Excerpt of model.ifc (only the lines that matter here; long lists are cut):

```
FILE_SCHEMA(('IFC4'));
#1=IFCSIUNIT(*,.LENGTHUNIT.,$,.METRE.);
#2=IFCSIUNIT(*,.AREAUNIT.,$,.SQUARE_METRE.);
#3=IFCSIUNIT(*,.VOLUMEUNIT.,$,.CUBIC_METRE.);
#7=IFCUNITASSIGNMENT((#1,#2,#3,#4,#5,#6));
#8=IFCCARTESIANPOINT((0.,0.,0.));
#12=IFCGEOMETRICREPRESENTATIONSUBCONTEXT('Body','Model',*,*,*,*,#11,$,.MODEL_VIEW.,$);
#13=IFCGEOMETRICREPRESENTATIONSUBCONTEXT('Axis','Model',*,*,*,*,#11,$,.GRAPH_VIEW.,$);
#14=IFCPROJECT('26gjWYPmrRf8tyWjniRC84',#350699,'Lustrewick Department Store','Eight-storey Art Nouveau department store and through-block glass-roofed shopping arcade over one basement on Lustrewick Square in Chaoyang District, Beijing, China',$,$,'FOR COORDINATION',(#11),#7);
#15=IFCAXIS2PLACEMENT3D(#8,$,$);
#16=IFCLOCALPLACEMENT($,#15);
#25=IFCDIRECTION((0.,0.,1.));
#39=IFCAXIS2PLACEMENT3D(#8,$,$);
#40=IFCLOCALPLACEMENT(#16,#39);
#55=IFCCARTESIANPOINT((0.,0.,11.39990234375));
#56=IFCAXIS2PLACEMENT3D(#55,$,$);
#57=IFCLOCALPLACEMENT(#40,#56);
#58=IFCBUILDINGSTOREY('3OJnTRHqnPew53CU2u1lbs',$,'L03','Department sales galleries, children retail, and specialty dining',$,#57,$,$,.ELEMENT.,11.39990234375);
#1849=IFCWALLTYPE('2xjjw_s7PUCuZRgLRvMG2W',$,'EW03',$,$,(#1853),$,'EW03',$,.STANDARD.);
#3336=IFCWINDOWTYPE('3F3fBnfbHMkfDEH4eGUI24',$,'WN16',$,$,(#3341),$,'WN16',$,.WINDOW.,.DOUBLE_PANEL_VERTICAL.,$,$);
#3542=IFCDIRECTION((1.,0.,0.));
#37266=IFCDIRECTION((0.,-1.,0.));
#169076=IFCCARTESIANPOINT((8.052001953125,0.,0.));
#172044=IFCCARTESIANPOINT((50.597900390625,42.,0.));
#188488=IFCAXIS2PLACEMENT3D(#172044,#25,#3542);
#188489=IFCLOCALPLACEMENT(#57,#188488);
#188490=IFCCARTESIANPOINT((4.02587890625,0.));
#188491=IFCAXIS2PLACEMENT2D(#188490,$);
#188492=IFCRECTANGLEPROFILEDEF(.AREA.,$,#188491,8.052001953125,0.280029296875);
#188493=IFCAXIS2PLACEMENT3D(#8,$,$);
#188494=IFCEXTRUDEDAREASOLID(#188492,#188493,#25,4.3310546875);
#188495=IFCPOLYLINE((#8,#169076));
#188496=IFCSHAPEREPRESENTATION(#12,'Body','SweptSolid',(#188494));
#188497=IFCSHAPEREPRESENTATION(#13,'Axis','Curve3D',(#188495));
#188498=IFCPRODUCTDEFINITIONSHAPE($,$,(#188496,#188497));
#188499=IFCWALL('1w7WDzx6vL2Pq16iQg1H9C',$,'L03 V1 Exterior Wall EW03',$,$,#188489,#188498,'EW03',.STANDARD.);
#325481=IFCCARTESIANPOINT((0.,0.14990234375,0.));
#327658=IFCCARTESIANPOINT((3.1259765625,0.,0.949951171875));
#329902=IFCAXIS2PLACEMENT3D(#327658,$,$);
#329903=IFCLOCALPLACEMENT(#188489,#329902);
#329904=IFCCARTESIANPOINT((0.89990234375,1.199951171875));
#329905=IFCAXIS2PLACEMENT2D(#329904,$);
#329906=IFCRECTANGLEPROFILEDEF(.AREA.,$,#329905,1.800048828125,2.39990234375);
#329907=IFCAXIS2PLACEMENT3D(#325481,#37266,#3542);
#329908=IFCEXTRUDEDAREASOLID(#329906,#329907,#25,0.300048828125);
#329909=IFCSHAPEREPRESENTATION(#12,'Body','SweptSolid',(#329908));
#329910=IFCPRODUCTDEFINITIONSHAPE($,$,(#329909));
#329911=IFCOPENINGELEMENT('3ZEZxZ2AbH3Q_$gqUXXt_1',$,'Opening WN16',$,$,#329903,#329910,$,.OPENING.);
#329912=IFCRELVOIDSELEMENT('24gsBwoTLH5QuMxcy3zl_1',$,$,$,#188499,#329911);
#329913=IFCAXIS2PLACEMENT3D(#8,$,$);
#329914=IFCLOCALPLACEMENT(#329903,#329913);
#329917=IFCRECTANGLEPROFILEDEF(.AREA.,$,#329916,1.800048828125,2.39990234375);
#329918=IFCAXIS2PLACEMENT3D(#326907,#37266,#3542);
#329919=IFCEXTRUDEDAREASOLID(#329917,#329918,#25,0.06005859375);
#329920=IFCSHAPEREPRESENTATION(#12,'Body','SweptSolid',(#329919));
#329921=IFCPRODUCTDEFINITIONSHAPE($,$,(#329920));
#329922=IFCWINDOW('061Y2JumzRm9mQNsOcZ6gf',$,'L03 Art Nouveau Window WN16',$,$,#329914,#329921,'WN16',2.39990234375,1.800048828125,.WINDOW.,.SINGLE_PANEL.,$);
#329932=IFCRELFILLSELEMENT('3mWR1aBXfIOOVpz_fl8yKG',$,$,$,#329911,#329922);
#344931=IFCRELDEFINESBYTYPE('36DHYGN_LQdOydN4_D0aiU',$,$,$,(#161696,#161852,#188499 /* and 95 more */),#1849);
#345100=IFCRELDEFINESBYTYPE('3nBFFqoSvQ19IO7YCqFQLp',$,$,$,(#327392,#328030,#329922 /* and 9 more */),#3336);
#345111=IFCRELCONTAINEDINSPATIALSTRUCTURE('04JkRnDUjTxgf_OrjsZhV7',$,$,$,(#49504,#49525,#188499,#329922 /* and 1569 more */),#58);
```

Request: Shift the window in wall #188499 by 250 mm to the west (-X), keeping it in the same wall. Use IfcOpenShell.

```python
import ifcopenshell
import ifcopenshell.api.geometry
import ifcopenshell.util.placement
import ifcopenshell.util.unit

model = ifcopenshell.open("model.ifc")
unit_scale = ifcopenshell.util.unit.calculate_unit_scale(model)

window = model.by_id(329922)
opening = window.FillsVoids[0].RelatingOpeningElement
wall = opening.VoidsElements[0].RelatingBuildingElement

wall_matrix = ifcopenshell.util.placement.get_local_placement(wall.ObjectPlacement)
shift = wall_matrix[:3, 0] * -0.25 / unit_scale
before = ifcopenshell.util.placement.get_local_placement(window.ObjectPlacement)[:3, 3].copy()

# The window is placed relative to its opening, so it follows when the opening moves.
matrix = ifcopenshell.util.placement.get_local_placement(opening.ObjectPlacement)
matrix[:3, 3] += shift
ifcopenshell.api.geometry.edit_object_placement(
    model, product=opening, matrix=matrix, is_si=False, should_transform_children=True
)

after = ifcopenshell.util.placement.get_local_placement(window.ObjectPlacement)[:3, 3]
print("window moved by", (after - before).round(3) + 0.0)

model.write("model_updated.ifc")
```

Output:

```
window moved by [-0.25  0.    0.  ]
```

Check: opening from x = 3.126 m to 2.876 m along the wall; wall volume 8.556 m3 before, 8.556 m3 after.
